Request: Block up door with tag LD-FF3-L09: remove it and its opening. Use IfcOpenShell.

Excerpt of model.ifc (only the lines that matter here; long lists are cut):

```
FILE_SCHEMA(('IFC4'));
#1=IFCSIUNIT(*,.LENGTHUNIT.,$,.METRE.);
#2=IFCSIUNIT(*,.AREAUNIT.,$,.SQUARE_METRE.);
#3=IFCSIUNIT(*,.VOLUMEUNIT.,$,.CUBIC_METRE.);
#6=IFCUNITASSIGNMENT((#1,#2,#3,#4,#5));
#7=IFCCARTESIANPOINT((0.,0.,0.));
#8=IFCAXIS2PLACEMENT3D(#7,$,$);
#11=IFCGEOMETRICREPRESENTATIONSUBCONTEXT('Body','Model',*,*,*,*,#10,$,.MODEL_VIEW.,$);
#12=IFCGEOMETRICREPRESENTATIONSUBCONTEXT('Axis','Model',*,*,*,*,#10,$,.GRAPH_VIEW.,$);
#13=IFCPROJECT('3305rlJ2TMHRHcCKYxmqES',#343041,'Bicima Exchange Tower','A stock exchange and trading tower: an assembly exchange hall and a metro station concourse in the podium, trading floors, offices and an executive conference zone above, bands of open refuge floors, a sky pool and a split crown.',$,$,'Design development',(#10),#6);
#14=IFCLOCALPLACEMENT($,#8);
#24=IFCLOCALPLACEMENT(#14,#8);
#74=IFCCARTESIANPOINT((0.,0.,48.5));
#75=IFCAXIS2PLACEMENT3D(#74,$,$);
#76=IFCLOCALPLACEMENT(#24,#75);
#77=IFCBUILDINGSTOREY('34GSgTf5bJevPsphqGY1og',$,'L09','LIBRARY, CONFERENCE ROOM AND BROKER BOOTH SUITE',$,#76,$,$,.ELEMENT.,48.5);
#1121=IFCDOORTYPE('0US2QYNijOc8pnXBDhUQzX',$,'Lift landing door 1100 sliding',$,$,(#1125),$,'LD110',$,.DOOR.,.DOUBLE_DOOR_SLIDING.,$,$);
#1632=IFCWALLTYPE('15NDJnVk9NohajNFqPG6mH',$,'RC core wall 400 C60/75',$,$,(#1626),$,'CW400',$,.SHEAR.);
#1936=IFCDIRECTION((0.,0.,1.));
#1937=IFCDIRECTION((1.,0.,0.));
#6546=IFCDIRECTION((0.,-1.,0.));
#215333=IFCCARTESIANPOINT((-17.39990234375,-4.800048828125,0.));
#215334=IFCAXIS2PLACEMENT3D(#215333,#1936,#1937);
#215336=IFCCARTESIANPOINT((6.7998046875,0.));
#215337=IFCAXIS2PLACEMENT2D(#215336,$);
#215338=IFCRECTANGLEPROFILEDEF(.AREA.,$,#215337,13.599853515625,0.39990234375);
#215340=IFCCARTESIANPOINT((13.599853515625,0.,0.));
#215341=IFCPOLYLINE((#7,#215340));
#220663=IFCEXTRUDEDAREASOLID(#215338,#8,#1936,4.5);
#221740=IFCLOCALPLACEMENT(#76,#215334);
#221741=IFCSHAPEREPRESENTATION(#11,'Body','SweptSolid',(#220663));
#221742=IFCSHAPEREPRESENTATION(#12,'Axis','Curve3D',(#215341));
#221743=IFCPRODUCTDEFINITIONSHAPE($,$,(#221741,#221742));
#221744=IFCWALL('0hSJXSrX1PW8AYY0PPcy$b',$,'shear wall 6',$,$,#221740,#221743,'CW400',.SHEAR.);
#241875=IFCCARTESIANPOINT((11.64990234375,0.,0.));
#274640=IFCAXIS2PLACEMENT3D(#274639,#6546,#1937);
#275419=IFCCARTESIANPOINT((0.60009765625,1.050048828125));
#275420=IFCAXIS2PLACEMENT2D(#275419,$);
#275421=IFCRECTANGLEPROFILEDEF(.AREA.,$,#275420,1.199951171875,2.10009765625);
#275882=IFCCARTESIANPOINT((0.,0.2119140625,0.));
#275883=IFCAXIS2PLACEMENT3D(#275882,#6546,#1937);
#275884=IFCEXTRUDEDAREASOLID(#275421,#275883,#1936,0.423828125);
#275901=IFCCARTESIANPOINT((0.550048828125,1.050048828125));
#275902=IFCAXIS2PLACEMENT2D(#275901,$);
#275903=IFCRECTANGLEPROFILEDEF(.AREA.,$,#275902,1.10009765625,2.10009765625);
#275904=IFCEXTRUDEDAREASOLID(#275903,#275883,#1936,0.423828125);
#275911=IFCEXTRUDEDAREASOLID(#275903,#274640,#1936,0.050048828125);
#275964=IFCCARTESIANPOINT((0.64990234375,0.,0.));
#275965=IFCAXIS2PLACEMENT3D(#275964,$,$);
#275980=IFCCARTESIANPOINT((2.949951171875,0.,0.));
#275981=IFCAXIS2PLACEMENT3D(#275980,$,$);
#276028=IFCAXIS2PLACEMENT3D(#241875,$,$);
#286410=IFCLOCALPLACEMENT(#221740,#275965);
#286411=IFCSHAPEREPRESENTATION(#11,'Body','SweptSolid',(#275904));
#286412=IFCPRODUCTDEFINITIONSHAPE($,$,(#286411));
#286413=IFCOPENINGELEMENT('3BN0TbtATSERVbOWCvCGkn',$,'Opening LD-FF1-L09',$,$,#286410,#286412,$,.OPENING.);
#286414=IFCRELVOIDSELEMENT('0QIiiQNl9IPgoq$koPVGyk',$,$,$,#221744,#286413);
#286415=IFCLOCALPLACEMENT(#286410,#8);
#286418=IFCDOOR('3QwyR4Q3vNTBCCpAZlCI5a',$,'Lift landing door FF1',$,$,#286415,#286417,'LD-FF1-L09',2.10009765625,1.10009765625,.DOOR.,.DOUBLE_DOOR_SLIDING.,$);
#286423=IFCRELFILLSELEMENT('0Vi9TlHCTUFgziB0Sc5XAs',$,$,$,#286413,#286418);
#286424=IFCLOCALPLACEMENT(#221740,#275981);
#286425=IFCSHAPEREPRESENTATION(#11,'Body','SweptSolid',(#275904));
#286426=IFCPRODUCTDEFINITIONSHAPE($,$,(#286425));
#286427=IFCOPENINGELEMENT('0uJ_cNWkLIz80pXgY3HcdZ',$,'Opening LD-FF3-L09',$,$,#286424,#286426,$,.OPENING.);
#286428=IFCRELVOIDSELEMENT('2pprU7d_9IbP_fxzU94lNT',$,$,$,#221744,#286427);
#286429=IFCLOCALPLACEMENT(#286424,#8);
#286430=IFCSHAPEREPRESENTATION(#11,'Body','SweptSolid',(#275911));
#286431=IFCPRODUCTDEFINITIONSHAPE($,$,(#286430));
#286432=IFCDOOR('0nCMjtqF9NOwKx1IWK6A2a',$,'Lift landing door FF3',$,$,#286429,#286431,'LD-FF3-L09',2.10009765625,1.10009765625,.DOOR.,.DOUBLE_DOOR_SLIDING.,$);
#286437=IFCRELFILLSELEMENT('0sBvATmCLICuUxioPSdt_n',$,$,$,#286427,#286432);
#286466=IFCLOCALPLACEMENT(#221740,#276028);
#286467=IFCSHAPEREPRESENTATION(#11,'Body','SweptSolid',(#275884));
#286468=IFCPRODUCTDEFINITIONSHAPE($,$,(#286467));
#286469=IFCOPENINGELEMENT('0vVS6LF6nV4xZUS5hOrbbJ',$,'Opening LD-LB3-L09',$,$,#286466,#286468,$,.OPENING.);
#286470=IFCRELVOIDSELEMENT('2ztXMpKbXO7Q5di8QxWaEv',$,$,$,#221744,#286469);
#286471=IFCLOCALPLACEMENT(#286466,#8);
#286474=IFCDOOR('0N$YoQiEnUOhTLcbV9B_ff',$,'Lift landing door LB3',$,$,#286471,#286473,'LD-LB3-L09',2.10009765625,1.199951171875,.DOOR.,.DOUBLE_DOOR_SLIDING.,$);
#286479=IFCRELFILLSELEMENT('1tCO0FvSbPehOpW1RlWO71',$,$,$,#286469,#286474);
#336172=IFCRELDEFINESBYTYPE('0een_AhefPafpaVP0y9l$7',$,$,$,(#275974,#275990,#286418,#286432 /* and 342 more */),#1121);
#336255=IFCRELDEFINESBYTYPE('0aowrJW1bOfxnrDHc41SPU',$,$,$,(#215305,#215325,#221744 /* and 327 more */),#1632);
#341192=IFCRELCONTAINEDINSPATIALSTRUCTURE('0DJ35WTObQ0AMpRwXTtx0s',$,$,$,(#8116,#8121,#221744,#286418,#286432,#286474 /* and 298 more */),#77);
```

```python
import ifcopenshell
import ifcopenshell.api.feature
import ifcopenshell.api.root
import ifcopenshell.geom
import ifcopenshell.util.shape

model = ifcopenshell.open("model.ifc")
settings = ifcopenshell.geom.settings()


def volume(element):
    """Net volume in cubic metres, openings subtracted."""
    shape = ifcopenshell.geom.create_shape(settings, element)
    return ifcopenshell.util.shape.get_volume(shape.geometry)


door = model.by_guid("0nCMjtqF9NOwKx1IWK6A2a")
opening = door.FillsVoids[0].RelatingOpeningElement
wall = opening.VoidsElements[0].RelatingBuildingElement
before = volume(wall)

ifcopenshell.api.root.remove_product(model, product=door)
ifcopenshell.api.feature.remove_feature(model, feature=opening)

after = volume(wall)

print(f"wall volume {before:.3f} -> {after:.3f} m3")

model.write("model_rev.ifc")
```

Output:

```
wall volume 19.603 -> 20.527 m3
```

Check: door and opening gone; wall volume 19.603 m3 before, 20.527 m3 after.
